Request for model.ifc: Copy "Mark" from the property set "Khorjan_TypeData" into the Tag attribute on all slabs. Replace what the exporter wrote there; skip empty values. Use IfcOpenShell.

First a look at what the model holds.

```python
import ifcopenshell
import ifcopenshell.util.element

model = ifcopenshell.open("model.ifc")
print(model.schema)
slabs = model.by_type("IfcSlab")
print(len(slabs), "slabs")
for e in slabs[:8]:
    source = ifcopenshell.util.element.get_pset(e, "Khorjan_TypeData", "Mark")
    target = e.Tag
    print(e.id(), repr(source), repr(target), sep=" | ")
```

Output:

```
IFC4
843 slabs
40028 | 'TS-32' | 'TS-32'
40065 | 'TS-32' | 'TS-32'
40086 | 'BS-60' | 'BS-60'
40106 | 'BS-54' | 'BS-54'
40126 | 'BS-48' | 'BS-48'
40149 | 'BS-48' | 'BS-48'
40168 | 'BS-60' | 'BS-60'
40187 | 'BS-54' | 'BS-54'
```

```python
import ifcopenshell
import ifcopenshell.util.element

model = ifcopenshell.open("model.ifc")

count = 0
for e in model.by_type("IfcSlab"):
    value = ifcopenshell.util.element.get_pset(e, "Khorjan_TypeData", "Mark")
    current = e.Tag
    if not value or not value.strip() or current == value:
        continue
    e.Tag = value
    count += 1

print(count, "slabs updated")

model.write("model-out.ifc")
```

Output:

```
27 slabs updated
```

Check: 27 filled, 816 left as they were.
